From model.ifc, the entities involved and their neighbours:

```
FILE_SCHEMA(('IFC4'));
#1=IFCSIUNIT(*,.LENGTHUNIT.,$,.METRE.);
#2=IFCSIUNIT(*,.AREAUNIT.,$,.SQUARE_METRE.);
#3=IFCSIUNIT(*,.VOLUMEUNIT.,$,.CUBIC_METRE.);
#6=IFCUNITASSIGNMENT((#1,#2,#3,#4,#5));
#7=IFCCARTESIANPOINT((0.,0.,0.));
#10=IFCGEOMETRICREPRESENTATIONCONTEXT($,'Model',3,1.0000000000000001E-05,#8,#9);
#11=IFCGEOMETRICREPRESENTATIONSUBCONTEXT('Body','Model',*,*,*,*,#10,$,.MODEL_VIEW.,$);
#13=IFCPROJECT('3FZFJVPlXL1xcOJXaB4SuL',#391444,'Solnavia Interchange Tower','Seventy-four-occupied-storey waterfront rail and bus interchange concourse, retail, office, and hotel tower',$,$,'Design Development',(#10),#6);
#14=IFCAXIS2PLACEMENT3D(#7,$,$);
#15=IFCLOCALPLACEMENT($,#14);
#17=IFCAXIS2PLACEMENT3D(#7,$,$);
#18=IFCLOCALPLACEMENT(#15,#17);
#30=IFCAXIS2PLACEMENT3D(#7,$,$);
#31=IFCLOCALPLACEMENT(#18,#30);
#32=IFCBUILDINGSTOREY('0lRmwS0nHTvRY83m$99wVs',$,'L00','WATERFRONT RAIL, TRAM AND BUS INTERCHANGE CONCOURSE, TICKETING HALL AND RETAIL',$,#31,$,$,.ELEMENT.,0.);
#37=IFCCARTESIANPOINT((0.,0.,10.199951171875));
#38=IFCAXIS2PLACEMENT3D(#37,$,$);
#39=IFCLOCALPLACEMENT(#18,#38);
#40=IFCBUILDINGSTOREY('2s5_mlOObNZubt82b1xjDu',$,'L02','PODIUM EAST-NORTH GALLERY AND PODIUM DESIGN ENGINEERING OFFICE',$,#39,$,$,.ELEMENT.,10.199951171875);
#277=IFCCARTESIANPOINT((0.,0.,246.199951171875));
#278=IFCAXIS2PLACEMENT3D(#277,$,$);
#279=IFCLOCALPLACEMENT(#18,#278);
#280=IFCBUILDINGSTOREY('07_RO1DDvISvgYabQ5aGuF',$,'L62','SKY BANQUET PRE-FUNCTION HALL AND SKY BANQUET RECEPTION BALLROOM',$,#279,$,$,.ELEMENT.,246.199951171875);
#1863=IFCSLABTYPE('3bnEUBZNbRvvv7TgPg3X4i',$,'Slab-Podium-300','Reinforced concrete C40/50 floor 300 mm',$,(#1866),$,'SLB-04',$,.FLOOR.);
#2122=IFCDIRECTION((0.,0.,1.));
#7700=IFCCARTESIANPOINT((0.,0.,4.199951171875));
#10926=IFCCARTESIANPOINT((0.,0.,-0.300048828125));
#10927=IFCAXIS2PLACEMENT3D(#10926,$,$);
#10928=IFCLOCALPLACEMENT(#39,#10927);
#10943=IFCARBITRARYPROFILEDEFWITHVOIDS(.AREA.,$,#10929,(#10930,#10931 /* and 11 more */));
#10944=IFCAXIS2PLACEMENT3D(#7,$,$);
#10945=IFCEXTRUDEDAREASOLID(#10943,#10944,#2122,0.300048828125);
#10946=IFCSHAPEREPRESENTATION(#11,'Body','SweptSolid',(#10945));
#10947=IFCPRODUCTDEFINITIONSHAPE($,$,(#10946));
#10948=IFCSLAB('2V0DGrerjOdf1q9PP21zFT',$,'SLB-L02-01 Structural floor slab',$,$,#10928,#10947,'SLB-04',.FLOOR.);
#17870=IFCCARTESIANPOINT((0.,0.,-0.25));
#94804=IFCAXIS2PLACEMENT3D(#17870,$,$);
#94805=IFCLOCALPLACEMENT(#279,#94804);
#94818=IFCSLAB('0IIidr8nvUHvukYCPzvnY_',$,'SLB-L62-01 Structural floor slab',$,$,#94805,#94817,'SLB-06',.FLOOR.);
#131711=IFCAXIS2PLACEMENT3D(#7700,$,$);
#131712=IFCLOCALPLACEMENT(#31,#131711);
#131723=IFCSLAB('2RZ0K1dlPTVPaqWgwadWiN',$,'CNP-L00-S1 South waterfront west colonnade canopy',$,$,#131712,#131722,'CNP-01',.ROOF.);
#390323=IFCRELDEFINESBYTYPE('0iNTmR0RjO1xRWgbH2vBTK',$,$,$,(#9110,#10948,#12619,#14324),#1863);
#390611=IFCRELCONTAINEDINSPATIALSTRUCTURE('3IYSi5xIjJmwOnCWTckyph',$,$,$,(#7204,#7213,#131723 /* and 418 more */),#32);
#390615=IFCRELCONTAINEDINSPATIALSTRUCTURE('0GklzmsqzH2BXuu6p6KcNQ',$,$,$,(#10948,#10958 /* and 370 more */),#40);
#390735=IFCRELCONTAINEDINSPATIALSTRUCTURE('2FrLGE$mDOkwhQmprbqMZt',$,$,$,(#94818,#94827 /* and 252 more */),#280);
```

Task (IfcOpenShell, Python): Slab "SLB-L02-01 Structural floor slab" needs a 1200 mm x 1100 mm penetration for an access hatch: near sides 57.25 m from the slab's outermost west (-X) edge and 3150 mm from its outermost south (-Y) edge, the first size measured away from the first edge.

```python
import numpy as np
import ifcopenshell
import ifcopenshell.api.feature
import ifcopenshell.api.geometry
import ifcopenshell.api.root
import ifcopenshell.geom
import ifcopenshell.util.placement
import ifcopenshell.util.representation
import ifcopenshell.util.shape
import ifcopenshell.util.unit

model = ifcopenshell.open("model.ifc")
unit_scale = ifcopenshell.util.unit.calculate_unit_scale(model)
settings = ifcopenshell.geom.settings()


def volume(element):
    """Net volume in cubic metres, openings subtracted."""
    shape = ifcopenshell.geom.create_shape(settings, element)
    return ifcopenshell.util.shape.get_volume(shape.geometry)


slab = model.by_id(10948)
before = volume(slab)

# Extent in the slab's own axes, in metres. The edges named are its -X and -Y sides.
slab_shape = ifcopenshell.geom.create_shape(settings, slab)
vertices = ifcopenshell.util.shape.get_vertices(slab_shape.geometry)
x_min, y_min, bottom = vertices.min(axis=0)
top = vertices[:, 2].max()

opening = ifcopenshell.api.root.create_entity(model, ifc_class="IfcOpeningElement", name="Access hatch opening", predefined_type="OPENING")
context = ifcopenshell.util.representation.get_context(model, "Model", "Body", "MODEL_VIEW")
width, depth = 1.2, 1.1
outline = [(0.0, 0.0), (width, 0.0), (width, depth), (0.0, depth), (0.0, 0.0)]
# Overshoot both faces by 50 mm so the cut is clean.
shape = ifcopenshell.api.geometry.add_slab_representation(
    model, context=context, depth=top - bottom + 0.1, polyline=outline
)
ifcopenshell.api.geometry.assign_representation(model, product=opening, representation=shape)

matrix = ifcopenshell.util.placement.get_local_placement(slab.ObjectPlacement)
matrix[:, 3] = matrix @ np.append(np.array([x_min + 57.25, y_min + 3.15, bottom - 0.05]) / unit_scale, 1.0)
ifcopenshell.api.geometry.edit_object_placement(model, product=opening, matrix=matrix, is_si=False)
ifcopenshell.api.feature.add_feature(model, feature=opening, element=slab)

after = volume(slab)

print(f"slab volume {before:.3f} -> {after:.3f} m3")

model.write("model_v2.ifc")
```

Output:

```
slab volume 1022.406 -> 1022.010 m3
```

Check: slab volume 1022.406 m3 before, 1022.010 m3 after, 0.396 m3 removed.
